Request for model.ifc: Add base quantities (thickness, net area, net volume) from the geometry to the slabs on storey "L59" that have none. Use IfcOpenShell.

First a look at what the model holds.

```python
import ifcopenshell
import ifcopenshell.util.element
import ifcopenshell.util.unit

model = ifcopenshell.open("model.ifc")
print(model.schema)
for unit_type in ("LENGTHUNIT", "AREAUNIT", "VOLUMEUNIT"):
    print(unit_type, ifcopenshell.util.unit.calculate_unit_scale(model, unit_type))
storey = next(s for s in model.by_type("IfcBuildingStorey") if s.Name == "L59")
slabs = [e for e in ifcopenshell.util.element.get_decomposition(storey) if e.is_a("IfcSlab")]
for e in sorted(slabs, key=lambda e: e.id()):
    print(e.id(), e.is_a(), e.Name, list(ifcopenshell.util.element.get_psets(e, qtos_only=True)), sep=" | ")
```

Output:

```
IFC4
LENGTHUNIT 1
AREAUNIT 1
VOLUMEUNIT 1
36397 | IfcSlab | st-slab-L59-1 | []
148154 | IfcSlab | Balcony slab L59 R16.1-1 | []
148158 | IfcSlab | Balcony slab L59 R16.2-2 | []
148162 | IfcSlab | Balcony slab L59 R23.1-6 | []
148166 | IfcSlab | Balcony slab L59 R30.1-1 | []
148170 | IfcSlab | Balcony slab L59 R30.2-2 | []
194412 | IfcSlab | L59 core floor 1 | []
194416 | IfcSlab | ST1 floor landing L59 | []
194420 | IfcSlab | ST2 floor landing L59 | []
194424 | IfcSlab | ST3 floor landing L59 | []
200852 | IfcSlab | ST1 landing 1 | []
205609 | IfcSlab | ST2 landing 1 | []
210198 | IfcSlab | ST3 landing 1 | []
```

```python
import ifcopenshell
import ifcopenshell.api.pset
import ifcopenshell.geom
import ifcopenshell.util.element
import ifcopenshell.util.shape
import ifcopenshell.util.unit

model = ifcopenshell.open("model.ifc")
unit_scale = ifcopenshell.util.unit.calculate_unit_scale(model)
area_scale = ifcopenshell.util.unit.calculate_unit_scale(model, "AREAUNIT")
volume_scale = ifcopenshell.util.unit.calculate_unit_scale(model, "VOLUMEUNIT")
settings = ifcopenshell.geom.settings()

storey = next(s for s in model.by_type("IfcBuildingStorey") if s.Name == "L59")
slabs = [e for e in ifcopenshell.util.element.get_decomposition(storey) if e.is_a("IfcSlab")]

for e in sorted(slabs, key=lambda e: e.id()):
    if ifcopenshell.util.element.get_psets(e, qtos_only=True, should_inherit=False):
        continue
    # Geometry comes back in metres, in the element's own axes.
    shape = ifcopenshell.geom.create_shape(settings, e)
    values = {
        "Width": ifcopenshell.util.shape.get_z(shape.geometry) / unit_scale,
        "NetArea": ifcopenshell.util.shape.get_footprint_area(shape.geometry) / area_scale,
        "NetVolume": ifcopenshell.util.shape.get_volume(shape.geometry) / volume_scale,
    }
    qto = ifcopenshell.api.pset.add_qto(model, product=e, name="Qto_SlabBaseQuantities")
    ifcopenshell.api.pset.edit_qto(model, qto=qto, properties=values)
    print(e.id(), {k: round(v, 3) for k, v in values.items()})

model.write("model_rev.ifc")
```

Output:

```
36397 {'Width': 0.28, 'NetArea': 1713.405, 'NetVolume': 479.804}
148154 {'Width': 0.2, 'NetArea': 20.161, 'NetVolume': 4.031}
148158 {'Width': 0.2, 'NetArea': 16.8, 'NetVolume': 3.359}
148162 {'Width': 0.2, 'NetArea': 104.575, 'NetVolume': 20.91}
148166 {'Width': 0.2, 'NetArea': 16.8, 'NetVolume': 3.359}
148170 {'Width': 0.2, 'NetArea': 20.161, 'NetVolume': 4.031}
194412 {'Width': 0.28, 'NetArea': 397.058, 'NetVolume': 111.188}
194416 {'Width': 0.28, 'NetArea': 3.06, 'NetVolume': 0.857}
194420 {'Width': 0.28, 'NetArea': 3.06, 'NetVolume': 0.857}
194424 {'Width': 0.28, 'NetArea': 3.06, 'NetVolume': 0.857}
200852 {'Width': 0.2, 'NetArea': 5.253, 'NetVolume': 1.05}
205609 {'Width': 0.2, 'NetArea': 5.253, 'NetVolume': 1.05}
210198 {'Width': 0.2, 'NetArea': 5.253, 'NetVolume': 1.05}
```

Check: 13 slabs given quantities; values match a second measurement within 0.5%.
